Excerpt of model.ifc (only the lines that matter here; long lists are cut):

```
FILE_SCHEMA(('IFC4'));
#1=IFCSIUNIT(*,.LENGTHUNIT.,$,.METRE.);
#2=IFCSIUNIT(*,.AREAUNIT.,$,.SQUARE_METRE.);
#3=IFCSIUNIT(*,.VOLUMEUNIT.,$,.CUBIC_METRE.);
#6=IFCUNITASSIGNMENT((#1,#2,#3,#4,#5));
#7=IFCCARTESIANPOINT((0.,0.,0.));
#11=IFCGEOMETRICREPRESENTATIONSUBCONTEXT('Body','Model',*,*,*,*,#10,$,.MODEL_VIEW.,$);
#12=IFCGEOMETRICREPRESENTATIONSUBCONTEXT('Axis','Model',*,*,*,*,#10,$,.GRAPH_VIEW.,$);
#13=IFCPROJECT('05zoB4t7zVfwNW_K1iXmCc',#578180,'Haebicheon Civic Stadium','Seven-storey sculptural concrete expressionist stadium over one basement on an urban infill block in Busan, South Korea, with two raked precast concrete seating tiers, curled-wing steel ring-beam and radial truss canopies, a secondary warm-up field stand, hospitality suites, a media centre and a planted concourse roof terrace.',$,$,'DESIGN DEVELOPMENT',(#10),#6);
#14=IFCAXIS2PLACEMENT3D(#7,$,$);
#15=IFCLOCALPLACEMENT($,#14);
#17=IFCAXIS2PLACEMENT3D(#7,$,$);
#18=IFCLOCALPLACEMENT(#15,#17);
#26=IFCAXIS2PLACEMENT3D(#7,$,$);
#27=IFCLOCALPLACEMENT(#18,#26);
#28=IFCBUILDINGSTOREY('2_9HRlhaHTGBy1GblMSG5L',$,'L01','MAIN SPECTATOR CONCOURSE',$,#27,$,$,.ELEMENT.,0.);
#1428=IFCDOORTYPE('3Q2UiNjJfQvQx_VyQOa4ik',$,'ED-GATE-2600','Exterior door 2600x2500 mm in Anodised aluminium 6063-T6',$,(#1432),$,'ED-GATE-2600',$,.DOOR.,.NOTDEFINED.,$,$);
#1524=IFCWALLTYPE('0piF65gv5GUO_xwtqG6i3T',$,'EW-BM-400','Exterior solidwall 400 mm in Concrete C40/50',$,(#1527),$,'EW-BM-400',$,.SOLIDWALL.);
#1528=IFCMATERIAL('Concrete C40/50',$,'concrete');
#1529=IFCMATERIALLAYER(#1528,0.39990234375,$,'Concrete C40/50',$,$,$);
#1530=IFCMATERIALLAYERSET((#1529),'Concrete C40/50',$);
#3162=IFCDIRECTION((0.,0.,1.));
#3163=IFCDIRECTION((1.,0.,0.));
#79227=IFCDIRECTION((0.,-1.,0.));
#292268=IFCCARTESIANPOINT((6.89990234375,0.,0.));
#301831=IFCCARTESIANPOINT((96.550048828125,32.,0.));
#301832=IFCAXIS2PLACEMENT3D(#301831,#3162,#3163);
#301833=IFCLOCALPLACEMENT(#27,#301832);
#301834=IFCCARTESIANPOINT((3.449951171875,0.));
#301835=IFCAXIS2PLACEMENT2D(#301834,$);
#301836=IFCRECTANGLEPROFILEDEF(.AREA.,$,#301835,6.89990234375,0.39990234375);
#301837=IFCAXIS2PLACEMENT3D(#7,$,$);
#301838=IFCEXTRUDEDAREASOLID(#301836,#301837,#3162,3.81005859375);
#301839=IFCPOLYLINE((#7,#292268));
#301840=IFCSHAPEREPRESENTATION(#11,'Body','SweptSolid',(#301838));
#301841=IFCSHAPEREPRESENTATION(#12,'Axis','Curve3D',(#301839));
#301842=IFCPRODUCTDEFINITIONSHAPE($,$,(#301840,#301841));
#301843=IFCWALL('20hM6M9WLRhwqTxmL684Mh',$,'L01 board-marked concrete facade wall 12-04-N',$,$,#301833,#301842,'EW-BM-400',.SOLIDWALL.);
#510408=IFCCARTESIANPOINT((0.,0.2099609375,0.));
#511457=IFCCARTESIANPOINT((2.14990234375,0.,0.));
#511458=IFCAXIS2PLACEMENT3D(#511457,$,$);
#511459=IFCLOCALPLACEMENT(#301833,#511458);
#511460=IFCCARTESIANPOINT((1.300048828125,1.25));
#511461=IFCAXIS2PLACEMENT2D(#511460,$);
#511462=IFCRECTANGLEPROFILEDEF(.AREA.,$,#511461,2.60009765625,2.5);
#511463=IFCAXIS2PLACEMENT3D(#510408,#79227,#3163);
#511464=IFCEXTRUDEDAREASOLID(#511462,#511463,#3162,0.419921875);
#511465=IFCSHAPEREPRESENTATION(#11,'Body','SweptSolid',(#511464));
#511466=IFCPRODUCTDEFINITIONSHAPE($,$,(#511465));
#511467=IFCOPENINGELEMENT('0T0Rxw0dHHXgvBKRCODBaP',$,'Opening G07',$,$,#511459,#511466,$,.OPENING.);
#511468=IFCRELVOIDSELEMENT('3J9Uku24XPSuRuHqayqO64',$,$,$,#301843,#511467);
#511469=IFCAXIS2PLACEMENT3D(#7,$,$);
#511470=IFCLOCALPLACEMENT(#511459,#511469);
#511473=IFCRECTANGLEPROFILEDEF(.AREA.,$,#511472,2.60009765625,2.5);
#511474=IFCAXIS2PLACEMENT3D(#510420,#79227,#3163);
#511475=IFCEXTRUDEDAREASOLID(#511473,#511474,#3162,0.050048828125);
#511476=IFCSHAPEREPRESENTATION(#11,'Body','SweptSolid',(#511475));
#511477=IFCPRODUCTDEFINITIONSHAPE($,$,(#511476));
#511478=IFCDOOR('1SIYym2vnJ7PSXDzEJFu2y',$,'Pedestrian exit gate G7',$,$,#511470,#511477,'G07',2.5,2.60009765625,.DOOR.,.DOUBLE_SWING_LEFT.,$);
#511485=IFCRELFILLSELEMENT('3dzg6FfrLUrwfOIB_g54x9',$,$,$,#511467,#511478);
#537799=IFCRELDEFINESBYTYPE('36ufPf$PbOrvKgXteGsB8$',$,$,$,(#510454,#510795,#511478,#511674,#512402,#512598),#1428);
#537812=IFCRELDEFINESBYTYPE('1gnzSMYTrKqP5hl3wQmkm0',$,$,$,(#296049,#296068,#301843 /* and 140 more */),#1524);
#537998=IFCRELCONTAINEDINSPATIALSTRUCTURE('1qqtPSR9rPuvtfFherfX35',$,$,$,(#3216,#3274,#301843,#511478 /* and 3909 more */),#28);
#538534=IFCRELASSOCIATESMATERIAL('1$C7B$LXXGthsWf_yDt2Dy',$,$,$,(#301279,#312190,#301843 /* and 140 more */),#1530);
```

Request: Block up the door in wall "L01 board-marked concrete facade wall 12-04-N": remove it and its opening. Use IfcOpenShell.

```python
import ifcopenshell
import ifcopenshell.api.feature
import ifcopenshell.api.root
import ifcopenshell.geom
import ifcopenshell.util.shape

model = ifcopenshell.open("model.ifc")
settings = ifcopenshell.geom.settings()


def volume(element):
    """Net volume in cubic metres, openings subtracted."""
    shape = ifcopenshell.geom.create_shape(settings, element)
    return ifcopenshell.util.shape.get_volume(shape.geometry)


door = model.by_guid("1SIYym2vnJ7PSXDzEJFu2y")
opening = door.FillsVoids[0].RelatingOpeningElement
wall = opening.VoidsElements[0].RelatingBuildingElement
before = volume(wall)

ifcopenshell.api.root.remove_product(model, product=door)
ifcopenshell.api.feature.remove_feature(model, feature=opening)

after = volume(wall)

print(f"wall volume {before:.3f} -> {after:.3f} m3")

model.write("model_rev.ifc")
```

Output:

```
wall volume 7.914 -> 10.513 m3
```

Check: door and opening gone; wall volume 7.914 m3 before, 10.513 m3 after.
